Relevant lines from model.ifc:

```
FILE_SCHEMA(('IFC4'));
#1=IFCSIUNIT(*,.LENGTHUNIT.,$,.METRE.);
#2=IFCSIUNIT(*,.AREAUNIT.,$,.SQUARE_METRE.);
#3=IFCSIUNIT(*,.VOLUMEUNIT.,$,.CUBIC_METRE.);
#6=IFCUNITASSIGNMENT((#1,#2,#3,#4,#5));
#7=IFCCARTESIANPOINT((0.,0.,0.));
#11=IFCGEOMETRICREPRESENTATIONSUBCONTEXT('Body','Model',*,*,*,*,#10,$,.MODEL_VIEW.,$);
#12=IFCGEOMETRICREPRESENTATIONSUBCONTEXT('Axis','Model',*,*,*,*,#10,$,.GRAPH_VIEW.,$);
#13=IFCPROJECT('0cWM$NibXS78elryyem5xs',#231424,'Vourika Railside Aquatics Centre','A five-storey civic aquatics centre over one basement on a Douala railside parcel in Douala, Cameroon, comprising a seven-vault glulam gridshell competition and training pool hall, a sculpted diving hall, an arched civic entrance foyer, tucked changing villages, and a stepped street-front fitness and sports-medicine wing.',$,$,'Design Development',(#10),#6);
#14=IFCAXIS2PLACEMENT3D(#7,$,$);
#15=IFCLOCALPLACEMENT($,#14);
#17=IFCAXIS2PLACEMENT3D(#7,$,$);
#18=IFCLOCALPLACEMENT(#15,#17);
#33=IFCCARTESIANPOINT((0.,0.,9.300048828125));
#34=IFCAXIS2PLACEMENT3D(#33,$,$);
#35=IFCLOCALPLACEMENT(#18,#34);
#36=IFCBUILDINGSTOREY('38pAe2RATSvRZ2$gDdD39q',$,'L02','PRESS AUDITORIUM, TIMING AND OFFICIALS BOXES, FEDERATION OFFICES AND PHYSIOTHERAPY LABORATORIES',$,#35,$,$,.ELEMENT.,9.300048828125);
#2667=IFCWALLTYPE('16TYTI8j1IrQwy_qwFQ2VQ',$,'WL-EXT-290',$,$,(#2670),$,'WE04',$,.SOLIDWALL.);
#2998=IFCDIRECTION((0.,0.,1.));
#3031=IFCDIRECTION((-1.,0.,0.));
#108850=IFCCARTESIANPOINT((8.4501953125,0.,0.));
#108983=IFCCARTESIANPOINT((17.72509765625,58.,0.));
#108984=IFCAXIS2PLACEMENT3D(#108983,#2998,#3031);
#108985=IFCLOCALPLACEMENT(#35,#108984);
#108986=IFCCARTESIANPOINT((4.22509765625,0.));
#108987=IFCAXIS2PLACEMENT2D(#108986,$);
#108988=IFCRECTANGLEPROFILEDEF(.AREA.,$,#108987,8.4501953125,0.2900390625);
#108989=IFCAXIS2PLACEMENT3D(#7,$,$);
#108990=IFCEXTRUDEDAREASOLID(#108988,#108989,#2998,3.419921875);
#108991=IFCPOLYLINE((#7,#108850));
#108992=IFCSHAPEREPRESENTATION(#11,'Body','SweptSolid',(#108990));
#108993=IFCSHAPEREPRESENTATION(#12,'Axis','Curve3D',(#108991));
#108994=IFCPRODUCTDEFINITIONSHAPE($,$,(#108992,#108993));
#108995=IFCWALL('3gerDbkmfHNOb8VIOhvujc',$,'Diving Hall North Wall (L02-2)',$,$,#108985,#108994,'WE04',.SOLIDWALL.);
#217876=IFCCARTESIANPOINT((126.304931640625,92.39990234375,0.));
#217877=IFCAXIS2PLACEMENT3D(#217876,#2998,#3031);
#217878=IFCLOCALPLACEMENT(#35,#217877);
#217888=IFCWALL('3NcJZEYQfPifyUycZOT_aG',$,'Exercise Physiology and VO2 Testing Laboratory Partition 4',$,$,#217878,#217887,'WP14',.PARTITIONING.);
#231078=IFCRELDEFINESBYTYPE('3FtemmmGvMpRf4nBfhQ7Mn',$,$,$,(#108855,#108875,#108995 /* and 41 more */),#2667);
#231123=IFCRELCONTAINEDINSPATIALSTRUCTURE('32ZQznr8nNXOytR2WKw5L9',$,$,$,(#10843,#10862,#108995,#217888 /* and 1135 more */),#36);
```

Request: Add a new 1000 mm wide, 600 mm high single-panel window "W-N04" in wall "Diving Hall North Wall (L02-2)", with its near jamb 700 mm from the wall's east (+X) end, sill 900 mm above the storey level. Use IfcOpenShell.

```python
import numpy as np
import ifcopenshell
import ifcopenshell.api.feature
import ifcopenshell.api.geometry
import ifcopenshell.api.root
import ifcopenshell.api.spatial
import ifcopenshell.geom
import ifcopenshell.util.element
import ifcopenshell.util.placement
import ifcopenshell.util.representation
import ifcopenshell.util.shape
import ifcopenshell.util.unit

model = ifcopenshell.open("model.ifc")
unit_scale = ifcopenshell.util.unit.calculate_unit_scale(model)
settings = ifcopenshell.geom.settings()


def volume(element):
    """Net volume in cubic metres, openings subtracted."""
    shape = ifcopenshell.geom.create_shape(settings, element)
    return ifcopenshell.util.shape.get_volume(shape.geometry)


wall = model.by_guid("3gerDbkmfHNOb8VIOhvujc")
storey = ifcopenshell.util.element.get_container(wall, ifc_class="IfcBuildingStorey")
context = ifcopenshell.util.representation.get_context(model, "Model", "Body", "MODEL_VIEW")
before = volume(wall)

width, height, from_end, sill = 1, 0.6, 0.7, 0.9  # metres

# The wall runs along its own X axis, and the end named is its -X end.
wall_shape = ifcopenshell.geom.create_shape(settings, wall)
x, y, z = ifcopenshell.util.shape.get_vertices(wall_shape.geometry).T
start = x.min() + from_end
face, thickness = float(y.min()), float(y.max() - y.min())
wall_matrix = ifcopenshell.util.placement.get_local_placement(wall.ObjectPlacement)
level = ifcopenshell.util.placement.get_local_placement(storey.ObjectPlacement)[2, 3]


def in_wall(x, y):
    """Placement at x, y metres in the wall's axes, at sill height."""
    matrix = wall_matrix.copy()
    matrix[:, 3] = wall_matrix @ np.array([x / unit_scale, y / unit_scale, 0.0, 1.0])
    matrix[2, 3] = level + sill / unit_scale
    return matrix


# Opening: a box that overshoots both wall faces by 50 mm.
opening = ifcopenshell.api.root.create_entity(model, ifc_class="IfcOpeningElement", predefined_type="OPENING")
box = ifcopenshell.api.geometry.add_wall_representation(
    model, context=context, length=width, height=height, thickness=thickness + 0.1
)
ifcopenshell.api.geometry.assign_representation(model, product=opening, representation=box)
ifcopenshell.api.geometry.edit_object_placement(model, product=opening, matrix=in_wall(start, face - 0.05), is_si=False)
ifcopenshell.api.feature.add_feature(model, feature=opening, element=wall)

window = ifcopenshell.api.root.create_entity(model, ifc_class="IfcWindow", name="W-N04", predefined_type="WINDOW")
window.OverallWidth, window.OverallHeight = width / unit_scale, height / unit_scale
window.PartitioningType = "SINGLE_PANEL"
body = ifcopenshell.api.geometry.add_window_representation(
    model,
    context=context,
    overall_width=window.OverallWidth,
    overall_height=window.OverallHeight,
    partition_type="SINGLE_PANEL",
)
ifcopenshell.api.geometry.assign_representation(model, product=window, representation=body)
ifcopenshell.api.spatial.assign_container(model, products=[window], relating_structure=storey)
ifcopenshell.api.feature.add_filling(model, opening=opening, element=window)

# Centre the window in the wall's thickness.
ifcopenshell.api.geometry.edit_object_placement(model, product=window, matrix=in_wall(start, face), is_si=False)
window_shape = ifcopenshell.geom.create_shape(settings, window)
depth = ifcopenshell.util.shape.get_vertices(window_shape.geometry)[:, 1]
offset = face + thickness / 2 - (depth.min() + depth.max()) / 2
ifcopenshell.api.geometry.edit_object_placement(model, product=window, matrix=in_wall(start, offset), is_si=False)

after = volume(wall)

print(f"wall volume {before:.3f} -> {after:.3f} m3")

model.write("model_updated.ifc")
```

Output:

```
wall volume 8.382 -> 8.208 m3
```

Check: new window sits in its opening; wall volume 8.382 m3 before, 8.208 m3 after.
